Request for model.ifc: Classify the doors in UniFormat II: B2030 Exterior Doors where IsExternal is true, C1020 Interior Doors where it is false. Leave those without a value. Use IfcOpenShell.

First a look at what the model holds.

```python
import ifcopenshell
import ifcopenshell.util.element

model = ifcopenshell.open("model.ifc")
print(model.schema)
print("classifications:", [c.Name for c in model.by_type("IfcClassification")])
values = [ifcopenshell.util.element.get_pset(e, "Pset_DoorCommon", "IsExternal") for e in model.by_type("IfcDoor")]
for value in (True, False, None):
    print("IsExternal", value, values.count(value))
```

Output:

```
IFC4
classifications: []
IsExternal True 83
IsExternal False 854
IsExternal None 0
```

```python
import ifcopenshell
import ifcopenshell.api.classification
import ifcopenshell.util.element

model = ifcopenshell.open("model.ifc")

system = ifcopenshell.api.classification.add_classification(model, classification="UniFormat II")

doors = model.by_type("IfcDoor")
external = {e: ifcopenshell.util.element.get_pset(e, "Pset_DoorCommon", "IsExternal") for e in doors}
for flag, code, name in ((True, "B2030", "Exterior Doors"), (False, "C1020", "Interior Doors")):
    products = [e for e in doors if external[e] is flag]
    ifcopenshell.api.classification.add_reference(
        model, products=products, classification=system, identification=code, name=name
    )
    print(code, len(products))

model.write("model_rev.ifc")
```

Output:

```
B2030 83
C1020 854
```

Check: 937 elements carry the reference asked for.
